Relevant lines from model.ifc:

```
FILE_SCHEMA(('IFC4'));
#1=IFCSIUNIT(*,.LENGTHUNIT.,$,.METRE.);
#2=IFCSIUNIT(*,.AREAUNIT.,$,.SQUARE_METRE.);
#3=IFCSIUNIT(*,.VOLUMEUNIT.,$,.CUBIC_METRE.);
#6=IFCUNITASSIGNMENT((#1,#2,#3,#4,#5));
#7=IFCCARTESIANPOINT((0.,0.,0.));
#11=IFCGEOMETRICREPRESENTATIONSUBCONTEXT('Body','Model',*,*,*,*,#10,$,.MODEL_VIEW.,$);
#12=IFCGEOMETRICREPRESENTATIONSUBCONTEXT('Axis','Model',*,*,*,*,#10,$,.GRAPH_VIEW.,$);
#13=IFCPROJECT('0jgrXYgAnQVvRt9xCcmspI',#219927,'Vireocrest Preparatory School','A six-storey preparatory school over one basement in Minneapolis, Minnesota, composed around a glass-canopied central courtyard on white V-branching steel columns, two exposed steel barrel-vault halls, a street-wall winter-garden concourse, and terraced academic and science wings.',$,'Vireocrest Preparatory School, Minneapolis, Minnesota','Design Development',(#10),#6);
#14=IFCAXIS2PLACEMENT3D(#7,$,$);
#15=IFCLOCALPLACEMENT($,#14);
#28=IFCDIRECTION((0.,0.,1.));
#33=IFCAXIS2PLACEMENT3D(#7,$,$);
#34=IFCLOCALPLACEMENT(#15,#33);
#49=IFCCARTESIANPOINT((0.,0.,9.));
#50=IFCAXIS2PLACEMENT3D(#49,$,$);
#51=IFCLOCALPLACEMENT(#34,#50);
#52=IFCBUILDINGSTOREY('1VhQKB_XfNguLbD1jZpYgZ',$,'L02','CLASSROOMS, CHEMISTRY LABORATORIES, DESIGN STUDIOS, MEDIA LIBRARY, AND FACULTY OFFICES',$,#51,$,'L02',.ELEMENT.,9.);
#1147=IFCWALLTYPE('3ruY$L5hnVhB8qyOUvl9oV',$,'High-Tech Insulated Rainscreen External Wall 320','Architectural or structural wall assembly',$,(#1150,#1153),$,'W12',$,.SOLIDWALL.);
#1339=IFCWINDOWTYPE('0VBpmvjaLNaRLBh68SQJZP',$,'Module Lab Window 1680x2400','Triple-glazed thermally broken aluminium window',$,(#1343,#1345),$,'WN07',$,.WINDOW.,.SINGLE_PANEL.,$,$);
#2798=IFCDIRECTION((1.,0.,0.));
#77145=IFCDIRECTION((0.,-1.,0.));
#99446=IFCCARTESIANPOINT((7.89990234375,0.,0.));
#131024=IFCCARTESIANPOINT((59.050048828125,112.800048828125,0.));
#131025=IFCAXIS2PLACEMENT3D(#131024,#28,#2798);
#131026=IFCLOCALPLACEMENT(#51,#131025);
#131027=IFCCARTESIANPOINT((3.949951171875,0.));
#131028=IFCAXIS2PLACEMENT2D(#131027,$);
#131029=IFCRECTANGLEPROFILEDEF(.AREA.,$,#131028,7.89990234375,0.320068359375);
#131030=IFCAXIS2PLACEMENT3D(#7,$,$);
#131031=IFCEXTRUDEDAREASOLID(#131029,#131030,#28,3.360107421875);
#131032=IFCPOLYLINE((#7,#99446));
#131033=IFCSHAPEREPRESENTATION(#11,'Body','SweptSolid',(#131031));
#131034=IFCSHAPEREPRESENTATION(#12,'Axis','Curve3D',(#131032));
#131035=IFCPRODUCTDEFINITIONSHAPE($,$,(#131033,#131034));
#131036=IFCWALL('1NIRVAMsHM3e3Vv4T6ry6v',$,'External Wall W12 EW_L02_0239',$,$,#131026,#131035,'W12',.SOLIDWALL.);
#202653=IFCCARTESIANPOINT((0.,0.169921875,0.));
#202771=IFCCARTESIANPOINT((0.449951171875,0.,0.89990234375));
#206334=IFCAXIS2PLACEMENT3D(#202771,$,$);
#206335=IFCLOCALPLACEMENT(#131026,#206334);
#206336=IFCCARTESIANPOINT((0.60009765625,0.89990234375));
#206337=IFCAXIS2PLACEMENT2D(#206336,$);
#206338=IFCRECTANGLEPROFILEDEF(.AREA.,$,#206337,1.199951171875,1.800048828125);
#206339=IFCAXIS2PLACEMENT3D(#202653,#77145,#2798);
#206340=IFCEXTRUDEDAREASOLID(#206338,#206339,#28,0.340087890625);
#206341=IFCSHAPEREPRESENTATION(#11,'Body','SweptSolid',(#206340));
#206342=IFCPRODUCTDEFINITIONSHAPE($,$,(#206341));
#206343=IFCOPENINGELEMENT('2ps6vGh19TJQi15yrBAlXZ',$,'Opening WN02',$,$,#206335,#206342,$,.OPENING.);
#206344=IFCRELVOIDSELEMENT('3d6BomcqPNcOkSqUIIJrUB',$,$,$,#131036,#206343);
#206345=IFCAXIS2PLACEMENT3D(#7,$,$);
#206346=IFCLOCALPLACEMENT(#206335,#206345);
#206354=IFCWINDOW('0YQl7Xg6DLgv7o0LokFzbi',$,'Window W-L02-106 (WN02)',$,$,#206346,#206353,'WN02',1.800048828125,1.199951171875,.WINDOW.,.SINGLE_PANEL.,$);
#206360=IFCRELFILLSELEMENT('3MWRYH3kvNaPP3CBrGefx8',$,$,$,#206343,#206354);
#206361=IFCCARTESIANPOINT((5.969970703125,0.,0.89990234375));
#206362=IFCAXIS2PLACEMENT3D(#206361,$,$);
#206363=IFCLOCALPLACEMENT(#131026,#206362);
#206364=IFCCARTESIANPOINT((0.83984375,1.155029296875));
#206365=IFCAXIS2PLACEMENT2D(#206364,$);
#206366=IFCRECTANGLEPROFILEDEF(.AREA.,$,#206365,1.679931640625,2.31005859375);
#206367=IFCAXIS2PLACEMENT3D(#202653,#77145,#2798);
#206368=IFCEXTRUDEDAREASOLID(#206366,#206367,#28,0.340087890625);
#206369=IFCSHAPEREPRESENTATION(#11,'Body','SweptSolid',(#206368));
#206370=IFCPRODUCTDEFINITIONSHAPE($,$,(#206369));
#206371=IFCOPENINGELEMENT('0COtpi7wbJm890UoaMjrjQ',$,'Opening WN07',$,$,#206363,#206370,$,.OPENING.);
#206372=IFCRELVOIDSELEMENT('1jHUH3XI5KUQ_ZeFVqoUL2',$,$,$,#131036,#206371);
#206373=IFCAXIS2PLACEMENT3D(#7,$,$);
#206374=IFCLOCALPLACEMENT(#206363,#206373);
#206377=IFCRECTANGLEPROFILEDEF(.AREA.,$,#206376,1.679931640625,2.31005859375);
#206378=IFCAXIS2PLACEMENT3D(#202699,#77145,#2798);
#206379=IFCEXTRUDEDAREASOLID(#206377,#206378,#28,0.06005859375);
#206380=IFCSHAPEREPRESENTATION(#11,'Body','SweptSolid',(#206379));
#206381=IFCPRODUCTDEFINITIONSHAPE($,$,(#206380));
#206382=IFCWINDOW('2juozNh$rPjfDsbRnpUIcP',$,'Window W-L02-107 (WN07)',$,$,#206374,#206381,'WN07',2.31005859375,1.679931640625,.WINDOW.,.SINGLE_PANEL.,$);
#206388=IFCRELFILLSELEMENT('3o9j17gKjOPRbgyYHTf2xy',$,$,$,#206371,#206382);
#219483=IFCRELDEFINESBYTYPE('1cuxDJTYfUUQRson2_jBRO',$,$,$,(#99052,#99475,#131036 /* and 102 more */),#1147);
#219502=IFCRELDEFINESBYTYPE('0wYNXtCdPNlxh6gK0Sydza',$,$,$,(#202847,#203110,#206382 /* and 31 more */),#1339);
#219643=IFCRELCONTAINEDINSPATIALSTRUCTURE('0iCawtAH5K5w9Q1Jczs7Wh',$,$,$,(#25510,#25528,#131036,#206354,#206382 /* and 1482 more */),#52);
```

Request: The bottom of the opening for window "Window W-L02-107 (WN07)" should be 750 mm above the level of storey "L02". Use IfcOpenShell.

```python
import numpy as np
import ifcopenshell
import ifcopenshell.api.geometry
import ifcopenshell.geom
import ifcopenshell.util.element
import ifcopenshell.util.placement
import ifcopenshell.util.shape
import ifcopenshell.util.unit

model = ifcopenshell.open("model.ifc")
unit_scale = ifcopenshell.util.unit.calculate_unit_scale(model)

window = model.by_guid("2juozNh$rPjfDsbRnpUIcP")
opening = window.FillsVoids[0].RelatingOpeningElement
storey = ifcopenshell.util.element.get_container(window, ifc_class="IfcBuildingStorey")
level = ifcopenshell.util.placement.get_local_placement(storey.ObjectPlacement)[2, 3]

# The opening's origin need not be at the sill, so measure its lowest point.
shape = ifcopenshell.geom.create_shape(ifcopenshell.geom.settings(), opening)
bottom = ifcopenshell.util.shape.get_shape_bottom_elevation(shape, shape.geometry) / unit_scale
dz = level + 0.75 / unit_scale - bottom

shift = np.array([0.0, 0.0, dz])
# The window is placed relative to its opening, so it follows when the opening moves.
matrix = ifcopenshell.util.placement.get_local_placement(opening.ObjectPlacement)
matrix[:3, 3] += shift
ifcopenshell.api.geometry.edit_object_placement(
    model, product=opening, matrix=matrix, is_si=False, should_transform_children=True
)

print(f"moved by {dz * unit_scale:+.3f} m")

model.write("model-out.ifc")
```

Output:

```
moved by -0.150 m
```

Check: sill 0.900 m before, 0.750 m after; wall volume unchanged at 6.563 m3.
